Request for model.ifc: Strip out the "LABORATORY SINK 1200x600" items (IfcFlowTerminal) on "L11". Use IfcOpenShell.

First a look at what the model holds.

```python
import ifcopenshell
import ifcopenshell.util.element

model = ifcopenshell.open("model.ifc")
print(model.schema)
storey = next(s for s in model.by_type("IfcBuildingStorey") if s.Name == "L11")
terminals = [e for e in ifcopenshell.util.element.get_decomposition(storey) if e.is_a("IfcFlowTerminal")]
seen = {}
for e in terminals:
    element_type = ifcopenshell.util.element.get_type(e)
    name = element_type.Name if element_type not in (None, e) else None
    seen[name] = seen.get(name, 0) + 1
for name, count in sorted(seen.items(), key=str):
    print(count, "x", name)
```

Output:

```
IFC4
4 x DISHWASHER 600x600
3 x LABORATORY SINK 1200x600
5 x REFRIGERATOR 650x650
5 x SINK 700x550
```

```python
import ifcopenshell
import ifcopenshell.api.root
import ifcopenshell.util.element

model = ifcopenshell.open("model.ifc")

storey = next(s for s in model.by_type("IfcBuildingStorey") if s.Name == "L11")
terminals = [e for e in ifcopenshell.util.element.get_decomposition(storey) if e.is_a("IfcFlowTerminal")]
targets = [e for e in terminals if (t := ifcopenshell.util.element.get_type(e)) not in (None, e) and t.Name == "LABORATORY SINK 1200x600"]

for e in targets:
    ifcopenshell.api.root.remove_product(model, product=e)
print(len(targets), "removed")

model.write("model-out.ifc")
```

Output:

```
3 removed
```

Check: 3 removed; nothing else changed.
